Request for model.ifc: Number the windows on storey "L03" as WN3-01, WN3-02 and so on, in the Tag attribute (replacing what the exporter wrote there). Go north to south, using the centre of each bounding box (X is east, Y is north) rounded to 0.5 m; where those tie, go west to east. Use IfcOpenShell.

First a look at what the model holds.

```python
import ifcopenshell
import ifcopenshell.util.element
import ifcopenshell.util.placement

model = ifcopenshell.open("model.ifc")
print(model.schema)
storey = next(s for s in model.by_type("IfcBuildingStorey") if s.Name == "L03")
windows = [e for e in ifcopenshell.util.element.get_decomposition(storey) if e.is_a("IfcWindow")]
for e in sorted(windows, key=lambda e: e.id()):
    origin = ifcopenshell.util.placement.get_local_placement(e.ObjectPlacement)[:3, 3]
    print(e.id(), e.Tag, e.Name, origin.round(2) + 0.0, sep=" | ")
```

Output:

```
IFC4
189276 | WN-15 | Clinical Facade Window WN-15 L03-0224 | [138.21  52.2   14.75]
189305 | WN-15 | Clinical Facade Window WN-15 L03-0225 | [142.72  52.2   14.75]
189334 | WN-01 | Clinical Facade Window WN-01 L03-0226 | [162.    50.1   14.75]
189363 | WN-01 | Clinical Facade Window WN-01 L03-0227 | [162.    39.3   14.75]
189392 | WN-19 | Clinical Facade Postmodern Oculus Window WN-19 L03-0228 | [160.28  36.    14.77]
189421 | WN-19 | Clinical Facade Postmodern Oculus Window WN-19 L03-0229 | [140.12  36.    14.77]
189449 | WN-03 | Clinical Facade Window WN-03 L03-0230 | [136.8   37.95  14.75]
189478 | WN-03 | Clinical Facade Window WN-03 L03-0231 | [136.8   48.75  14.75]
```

```python
import ifcopenshell
import ifcopenshell.geom
import ifcopenshell.util.element
import ifcopenshell.util.shape

model = ifcopenshell.open("model.ifc")
settings = ifcopenshell.geom.settings()
settings.set("use-world-coords", True)


def centre(element):
    shape = ifcopenshell.geom.create_shape(settings, element)
    return ifcopenshell.util.shape.get_bbox_centroid(shape.geometry)


storey = next(s for s in model.by_type("IfcBuildingStorey") if s.Name == "L03")
windows = [e for e in ifcopenshell.util.element.get_decomposition(storey) if e.is_a("IfcWindow")]

# Insertion points can sit at a corner or the storey origin, so sort by the geometry (in metres).
centres = {e: centre(e) for e in windows}
windows.sort(key=lambda e: (-round(centres[e][1] / 0.5), centres[e][0]))

for i, e in enumerate(windows, start=1):
    number = f"WN3-{i:02d}"
    e.Tag = number
    print(e.id(), number)

model.write("model_rev.ifc")
```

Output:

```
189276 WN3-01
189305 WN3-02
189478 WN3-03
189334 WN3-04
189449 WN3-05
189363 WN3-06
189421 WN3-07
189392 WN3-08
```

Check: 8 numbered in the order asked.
